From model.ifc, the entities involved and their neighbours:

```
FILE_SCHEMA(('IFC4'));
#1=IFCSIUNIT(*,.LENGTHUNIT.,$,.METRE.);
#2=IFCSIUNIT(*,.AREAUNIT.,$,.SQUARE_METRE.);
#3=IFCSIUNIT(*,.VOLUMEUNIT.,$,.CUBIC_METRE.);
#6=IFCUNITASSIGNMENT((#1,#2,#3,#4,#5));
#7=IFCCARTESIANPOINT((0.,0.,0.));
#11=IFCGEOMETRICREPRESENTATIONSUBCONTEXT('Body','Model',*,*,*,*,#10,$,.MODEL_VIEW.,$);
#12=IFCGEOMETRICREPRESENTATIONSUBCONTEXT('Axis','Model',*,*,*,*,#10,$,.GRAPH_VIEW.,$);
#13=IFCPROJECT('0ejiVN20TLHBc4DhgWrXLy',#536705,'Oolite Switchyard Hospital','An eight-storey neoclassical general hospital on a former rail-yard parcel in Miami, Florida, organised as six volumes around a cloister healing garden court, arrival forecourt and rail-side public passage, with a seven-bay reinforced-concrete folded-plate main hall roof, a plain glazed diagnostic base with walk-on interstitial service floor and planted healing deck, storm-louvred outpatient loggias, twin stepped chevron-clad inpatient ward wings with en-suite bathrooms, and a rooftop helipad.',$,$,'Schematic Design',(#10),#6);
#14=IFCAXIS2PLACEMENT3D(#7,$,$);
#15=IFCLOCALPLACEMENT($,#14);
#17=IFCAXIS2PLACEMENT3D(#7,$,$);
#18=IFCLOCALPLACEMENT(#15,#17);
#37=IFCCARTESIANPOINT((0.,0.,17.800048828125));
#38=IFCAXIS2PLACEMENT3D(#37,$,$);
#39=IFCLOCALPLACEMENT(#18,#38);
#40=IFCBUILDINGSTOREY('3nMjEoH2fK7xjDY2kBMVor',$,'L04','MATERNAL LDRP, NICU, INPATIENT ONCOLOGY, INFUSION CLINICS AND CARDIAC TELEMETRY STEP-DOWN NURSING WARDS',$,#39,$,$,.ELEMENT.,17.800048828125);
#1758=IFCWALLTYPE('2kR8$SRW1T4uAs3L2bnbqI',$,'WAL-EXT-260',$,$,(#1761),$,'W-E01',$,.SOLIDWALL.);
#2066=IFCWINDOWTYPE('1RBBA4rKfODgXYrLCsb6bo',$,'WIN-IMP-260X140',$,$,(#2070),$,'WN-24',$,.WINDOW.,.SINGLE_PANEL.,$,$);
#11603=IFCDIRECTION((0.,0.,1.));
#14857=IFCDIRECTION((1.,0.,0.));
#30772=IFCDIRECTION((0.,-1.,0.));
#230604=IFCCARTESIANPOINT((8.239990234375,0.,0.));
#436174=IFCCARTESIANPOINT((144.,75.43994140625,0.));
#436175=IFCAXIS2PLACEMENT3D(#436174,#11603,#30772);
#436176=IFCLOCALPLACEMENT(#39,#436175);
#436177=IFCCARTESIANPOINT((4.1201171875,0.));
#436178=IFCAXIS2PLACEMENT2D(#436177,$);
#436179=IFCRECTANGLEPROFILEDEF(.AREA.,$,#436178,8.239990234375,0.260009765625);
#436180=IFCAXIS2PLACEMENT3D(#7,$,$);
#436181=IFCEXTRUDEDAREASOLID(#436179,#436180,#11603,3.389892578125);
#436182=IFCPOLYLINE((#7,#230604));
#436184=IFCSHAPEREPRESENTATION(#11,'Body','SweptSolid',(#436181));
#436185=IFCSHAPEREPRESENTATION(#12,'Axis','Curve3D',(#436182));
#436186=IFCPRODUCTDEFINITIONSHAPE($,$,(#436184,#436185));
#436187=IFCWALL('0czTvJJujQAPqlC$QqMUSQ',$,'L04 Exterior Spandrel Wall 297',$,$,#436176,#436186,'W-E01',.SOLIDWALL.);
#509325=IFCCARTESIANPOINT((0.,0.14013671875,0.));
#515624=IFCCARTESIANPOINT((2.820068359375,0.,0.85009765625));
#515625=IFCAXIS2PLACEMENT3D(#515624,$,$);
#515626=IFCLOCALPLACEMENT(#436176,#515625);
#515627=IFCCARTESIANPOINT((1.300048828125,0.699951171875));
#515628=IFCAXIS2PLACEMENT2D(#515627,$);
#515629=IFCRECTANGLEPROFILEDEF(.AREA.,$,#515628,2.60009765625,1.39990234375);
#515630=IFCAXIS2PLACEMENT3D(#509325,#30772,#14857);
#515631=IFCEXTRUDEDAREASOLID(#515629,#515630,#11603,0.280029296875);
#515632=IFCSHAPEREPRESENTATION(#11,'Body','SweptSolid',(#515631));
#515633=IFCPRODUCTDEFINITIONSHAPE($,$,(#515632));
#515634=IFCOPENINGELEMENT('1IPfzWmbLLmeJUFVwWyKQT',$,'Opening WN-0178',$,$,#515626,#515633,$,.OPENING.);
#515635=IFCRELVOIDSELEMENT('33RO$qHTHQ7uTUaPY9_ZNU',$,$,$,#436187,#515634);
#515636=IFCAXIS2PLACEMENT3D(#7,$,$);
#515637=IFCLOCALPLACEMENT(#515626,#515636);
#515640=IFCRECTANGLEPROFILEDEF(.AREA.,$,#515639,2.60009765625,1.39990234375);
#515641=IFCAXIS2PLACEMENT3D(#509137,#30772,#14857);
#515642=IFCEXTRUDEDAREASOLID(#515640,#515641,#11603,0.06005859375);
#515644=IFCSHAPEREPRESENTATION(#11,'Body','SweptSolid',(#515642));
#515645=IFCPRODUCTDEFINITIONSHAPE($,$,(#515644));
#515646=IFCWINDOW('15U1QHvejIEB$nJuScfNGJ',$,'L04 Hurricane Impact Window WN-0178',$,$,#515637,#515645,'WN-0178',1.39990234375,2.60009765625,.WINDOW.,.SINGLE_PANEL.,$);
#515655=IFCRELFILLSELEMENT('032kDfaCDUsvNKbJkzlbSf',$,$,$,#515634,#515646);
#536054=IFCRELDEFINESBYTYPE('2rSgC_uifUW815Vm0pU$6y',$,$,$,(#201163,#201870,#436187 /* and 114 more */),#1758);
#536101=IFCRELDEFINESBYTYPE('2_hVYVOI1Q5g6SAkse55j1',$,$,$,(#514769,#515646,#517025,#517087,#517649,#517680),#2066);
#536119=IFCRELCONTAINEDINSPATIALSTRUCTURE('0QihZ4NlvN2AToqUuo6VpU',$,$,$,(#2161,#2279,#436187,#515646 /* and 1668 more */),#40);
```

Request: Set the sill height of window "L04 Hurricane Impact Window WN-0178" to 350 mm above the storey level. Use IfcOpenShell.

```python
import numpy as np
import ifcopenshell
import ifcopenshell.api.geometry
import ifcopenshell.geom
import ifcopenshell.util.element
import ifcopenshell.util.placement
import ifcopenshell.util.shape
import ifcopenshell.util.unit

model = ifcopenshell.open("model.ifc")
unit_scale = ifcopenshell.util.unit.calculate_unit_scale(model)

window = model.by_guid("15U1QHvejIEB$nJuScfNGJ")
opening = window.FillsVoids[0].RelatingOpeningElement
storey = ifcopenshell.util.element.get_container(window, ifc_class="IfcBuildingStorey")
level = ifcopenshell.util.placement.get_local_placement(storey.ObjectPlacement)[2, 3]

# The opening's origin need not be at the sill, so measure its lowest point.
shape = ifcopenshell.geom.create_shape(ifcopenshell.geom.settings(), opening)
bottom = ifcopenshell.util.shape.get_shape_bottom_elevation(shape, shape.geometry) / unit_scale
dz = level + 0.35 / unit_scale - bottom

shift = np.array([0.0, 0.0, dz])
# The window is placed relative to its opening, so it follows when the opening moves.
matrix = ifcopenshell.util.placement.get_local_placement(opening.ObjectPlacement)
matrix[:3, 3] += shift
ifcopenshell.api.geometry.edit_object_placement(
    model, product=opening, matrix=matrix, is_si=False, should_transform_children=True
)

print(f"moved by {dz * unit_scale:+.3f} m")

model.write("model_rev.ifc")
```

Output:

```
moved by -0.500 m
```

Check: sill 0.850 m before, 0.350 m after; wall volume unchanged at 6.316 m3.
